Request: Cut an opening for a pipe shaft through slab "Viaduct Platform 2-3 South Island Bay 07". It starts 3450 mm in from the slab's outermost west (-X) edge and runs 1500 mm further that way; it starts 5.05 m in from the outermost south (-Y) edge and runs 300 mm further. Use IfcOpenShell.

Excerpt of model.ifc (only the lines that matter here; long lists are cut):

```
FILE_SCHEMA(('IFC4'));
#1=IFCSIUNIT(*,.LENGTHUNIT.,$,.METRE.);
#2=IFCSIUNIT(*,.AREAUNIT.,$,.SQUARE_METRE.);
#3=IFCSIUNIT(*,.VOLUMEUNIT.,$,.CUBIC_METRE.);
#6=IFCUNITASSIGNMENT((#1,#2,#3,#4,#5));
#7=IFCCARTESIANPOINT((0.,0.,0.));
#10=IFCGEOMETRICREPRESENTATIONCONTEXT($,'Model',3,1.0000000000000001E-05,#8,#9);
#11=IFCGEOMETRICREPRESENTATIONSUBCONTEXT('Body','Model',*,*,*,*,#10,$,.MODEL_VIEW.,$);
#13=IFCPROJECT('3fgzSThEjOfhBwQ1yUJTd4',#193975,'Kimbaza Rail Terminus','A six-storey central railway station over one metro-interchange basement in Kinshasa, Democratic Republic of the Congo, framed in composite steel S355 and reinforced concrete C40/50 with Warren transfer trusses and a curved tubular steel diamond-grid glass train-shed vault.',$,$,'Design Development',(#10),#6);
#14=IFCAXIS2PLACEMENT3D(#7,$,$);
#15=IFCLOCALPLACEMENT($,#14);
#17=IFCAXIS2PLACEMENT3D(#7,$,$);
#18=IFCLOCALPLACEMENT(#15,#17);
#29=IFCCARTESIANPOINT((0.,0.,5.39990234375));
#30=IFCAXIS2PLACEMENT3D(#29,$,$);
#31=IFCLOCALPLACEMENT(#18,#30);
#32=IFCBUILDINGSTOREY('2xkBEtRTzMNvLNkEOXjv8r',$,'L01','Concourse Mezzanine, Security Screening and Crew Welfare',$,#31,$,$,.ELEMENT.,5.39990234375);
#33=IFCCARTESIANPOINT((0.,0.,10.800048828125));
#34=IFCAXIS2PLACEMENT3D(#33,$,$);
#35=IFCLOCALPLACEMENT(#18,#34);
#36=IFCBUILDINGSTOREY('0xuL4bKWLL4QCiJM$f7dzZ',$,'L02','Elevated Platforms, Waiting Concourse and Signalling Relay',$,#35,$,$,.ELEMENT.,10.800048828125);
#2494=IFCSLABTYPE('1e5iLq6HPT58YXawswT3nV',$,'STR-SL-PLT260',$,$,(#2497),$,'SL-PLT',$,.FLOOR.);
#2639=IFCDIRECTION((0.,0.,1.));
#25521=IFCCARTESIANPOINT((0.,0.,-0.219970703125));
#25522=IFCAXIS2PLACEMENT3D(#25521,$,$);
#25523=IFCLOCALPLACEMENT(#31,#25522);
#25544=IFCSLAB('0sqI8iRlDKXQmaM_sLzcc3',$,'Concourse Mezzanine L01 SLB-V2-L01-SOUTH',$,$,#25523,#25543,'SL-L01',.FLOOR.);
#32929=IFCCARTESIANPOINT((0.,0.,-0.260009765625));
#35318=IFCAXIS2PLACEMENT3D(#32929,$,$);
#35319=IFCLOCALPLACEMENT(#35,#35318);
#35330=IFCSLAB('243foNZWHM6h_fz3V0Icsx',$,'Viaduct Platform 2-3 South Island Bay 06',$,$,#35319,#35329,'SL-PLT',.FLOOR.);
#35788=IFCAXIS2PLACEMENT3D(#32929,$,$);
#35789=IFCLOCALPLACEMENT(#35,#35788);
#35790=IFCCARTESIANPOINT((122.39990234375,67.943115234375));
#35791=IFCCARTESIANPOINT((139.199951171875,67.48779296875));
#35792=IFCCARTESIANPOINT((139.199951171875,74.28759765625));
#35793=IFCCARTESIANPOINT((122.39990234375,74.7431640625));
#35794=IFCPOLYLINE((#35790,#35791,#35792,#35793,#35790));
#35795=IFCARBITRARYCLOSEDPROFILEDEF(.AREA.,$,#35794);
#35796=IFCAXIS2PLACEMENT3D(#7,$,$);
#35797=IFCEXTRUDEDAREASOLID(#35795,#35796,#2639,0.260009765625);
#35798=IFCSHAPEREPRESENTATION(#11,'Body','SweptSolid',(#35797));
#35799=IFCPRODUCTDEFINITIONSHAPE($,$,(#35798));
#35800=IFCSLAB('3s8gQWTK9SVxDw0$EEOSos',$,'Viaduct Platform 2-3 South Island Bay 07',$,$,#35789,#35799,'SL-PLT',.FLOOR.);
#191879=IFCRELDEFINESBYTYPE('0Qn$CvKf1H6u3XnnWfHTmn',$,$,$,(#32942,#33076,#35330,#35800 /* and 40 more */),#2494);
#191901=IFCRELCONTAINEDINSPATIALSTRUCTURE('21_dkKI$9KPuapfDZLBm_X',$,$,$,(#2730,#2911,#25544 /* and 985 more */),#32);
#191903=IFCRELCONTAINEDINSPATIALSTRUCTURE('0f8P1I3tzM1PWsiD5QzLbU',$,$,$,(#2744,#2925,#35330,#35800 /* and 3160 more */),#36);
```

```python
import numpy as np
import ifcopenshell
import ifcopenshell.api.feature
import ifcopenshell.api.geometry
import ifcopenshell.api.root
import ifcopenshell.geom
import ifcopenshell.util.placement
import ifcopenshell.util.representation
import ifcopenshell.util.shape
import ifcopenshell.util.unit

model = ifcopenshell.open("model.ifc")
unit_scale = ifcopenshell.util.unit.calculate_unit_scale(model)
settings = ifcopenshell.geom.settings()


def volume(element):
    """Net volume in cubic metres, openings subtracted."""
    shape = ifcopenshell.geom.create_shape(settings, element)
    return ifcopenshell.util.shape.get_volume(shape.geometry)


slab = model.by_guid("3s8gQWTK9SVxDw0$EEOSos")
before = volume(slab)

# Extent in the slab's own axes, in metres. The edges named are its -X and -Y sides.
slab_shape = ifcopenshell.geom.create_shape(settings, slab)
vertices = ifcopenshell.util.shape.get_vertices(slab_shape.geometry)
x_min, y_min, bottom = vertices.min(axis=0)
top = vertices[:, 2].max()

opening = ifcopenshell.api.root.create_entity(model, ifc_class="IfcOpeningElement", name="Pipe shaft opening", predefined_type="OPENING")
context = ifcopenshell.util.representation.get_context(model, "Model", "Body", "MODEL_VIEW")
width, depth = 1.5, 0.3
outline = [(0.0, 0.0), (width, 0.0), (width, depth), (0.0, depth), (0.0, 0.0)]
# Overshoot both faces by 50 mm so the cut is clean.
shape = ifcopenshell.api.geometry.add_slab_representation(
    model, context=context, depth=top - bottom + 0.1, polyline=outline
)
ifcopenshell.api.geometry.assign_representation(model, product=opening, representation=shape)

matrix = ifcopenshell.util.placement.get_local_placement(slab.ObjectPlacement)
matrix[:, 3] = matrix @ np.append(np.array([x_min + 3.45, y_min + 5.05, bottom - 0.05]) / unit_scale, 1.0)
ifcopenshell.api.geometry.edit_object_placement(model, product=opening, matrix=matrix, is_si=False)
ifcopenshell.api.feature.add_feature(model, feature=opening, element=slab)

after = volume(slab)

print(f"slab volume {before:.3f} -> {after:.3f} m3")

model.write("model_updated.ifc")
```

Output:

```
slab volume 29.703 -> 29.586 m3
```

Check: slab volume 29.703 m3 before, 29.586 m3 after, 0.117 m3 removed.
